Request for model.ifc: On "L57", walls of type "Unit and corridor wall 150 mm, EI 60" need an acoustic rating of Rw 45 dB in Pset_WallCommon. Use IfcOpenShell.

First a look at what the model holds.

```python
import ifcopenshell
import ifcopenshell.util.element

model = ifcopenshell.open("model.ifc")
print(model.schema)
storey = next(s for s in model.by_type("IfcBuildingStorey") if s.Name == "L57")
walls = [e for e in ifcopenshell.util.element.get_decomposition(storey) if e.is_a("IfcWall")]
seen = {}
for e in walls:
    element_type = ifcopenshell.util.element.get_type(e)
    key = (element_type.Name if element_type != e and element_type else None, ifcopenshell.util.element.get_pset(e, "Pset_WallCommon", "AcousticRating"))
    seen[key] = seen.get(key, 0) + 1
for (name, value), count in sorted(seen.items(), key=str):
    print(count, "x", name, "|", value)
```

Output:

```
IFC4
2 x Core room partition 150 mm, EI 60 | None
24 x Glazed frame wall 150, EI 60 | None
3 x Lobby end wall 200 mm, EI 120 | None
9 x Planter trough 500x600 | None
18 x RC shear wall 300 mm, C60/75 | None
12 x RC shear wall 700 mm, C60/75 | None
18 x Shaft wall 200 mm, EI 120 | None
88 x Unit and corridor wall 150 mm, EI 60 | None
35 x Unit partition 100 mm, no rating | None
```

```python
import ifcopenshell
import ifcopenshell.api.pset
import ifcopenshell.util.element

model = ifcopenshell.open("model.ifc")

storey = next(s for s in model.by_type("IfcBuildingStorey") if s.Name == "L57")
walls = [e for e in ifcopenshell.util.element.get_decomposition(storey) if e.is_a("IfcWall")]

count = 0
for e in walls:
    element_type = ifcopenshell.util.element.get_type(e)
    if element_type in (None, e) or element_type.Name != "Unit and corridor wall 150 mm, EI 60":
        continue
    found = ifcopenshell.util.element.get_pset(e, "Pset_WallCommon", should_inherit=False)
    if found:
        pset = model.by_id(found["id"])
        if len(ifcopenshell.util.element.get_elements_by_pset(pset)) > 1:
            pset = ifcopenshell.api.pset.unshare_pset(model, products=[e], pset=pset)[0]
    else:
        pset = ifcopenshell.api.pset.add_pset(model, product=e, name="Pset_WallCommon")
    ifcopenshell.api.pset.edit_pset(model, pset=pset, properties={"AcousticRating": "Rw 45 dB"})
    count += 1

print(count, "walls updated")

model.write("model_edited.ifc")
```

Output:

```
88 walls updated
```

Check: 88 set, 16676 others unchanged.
